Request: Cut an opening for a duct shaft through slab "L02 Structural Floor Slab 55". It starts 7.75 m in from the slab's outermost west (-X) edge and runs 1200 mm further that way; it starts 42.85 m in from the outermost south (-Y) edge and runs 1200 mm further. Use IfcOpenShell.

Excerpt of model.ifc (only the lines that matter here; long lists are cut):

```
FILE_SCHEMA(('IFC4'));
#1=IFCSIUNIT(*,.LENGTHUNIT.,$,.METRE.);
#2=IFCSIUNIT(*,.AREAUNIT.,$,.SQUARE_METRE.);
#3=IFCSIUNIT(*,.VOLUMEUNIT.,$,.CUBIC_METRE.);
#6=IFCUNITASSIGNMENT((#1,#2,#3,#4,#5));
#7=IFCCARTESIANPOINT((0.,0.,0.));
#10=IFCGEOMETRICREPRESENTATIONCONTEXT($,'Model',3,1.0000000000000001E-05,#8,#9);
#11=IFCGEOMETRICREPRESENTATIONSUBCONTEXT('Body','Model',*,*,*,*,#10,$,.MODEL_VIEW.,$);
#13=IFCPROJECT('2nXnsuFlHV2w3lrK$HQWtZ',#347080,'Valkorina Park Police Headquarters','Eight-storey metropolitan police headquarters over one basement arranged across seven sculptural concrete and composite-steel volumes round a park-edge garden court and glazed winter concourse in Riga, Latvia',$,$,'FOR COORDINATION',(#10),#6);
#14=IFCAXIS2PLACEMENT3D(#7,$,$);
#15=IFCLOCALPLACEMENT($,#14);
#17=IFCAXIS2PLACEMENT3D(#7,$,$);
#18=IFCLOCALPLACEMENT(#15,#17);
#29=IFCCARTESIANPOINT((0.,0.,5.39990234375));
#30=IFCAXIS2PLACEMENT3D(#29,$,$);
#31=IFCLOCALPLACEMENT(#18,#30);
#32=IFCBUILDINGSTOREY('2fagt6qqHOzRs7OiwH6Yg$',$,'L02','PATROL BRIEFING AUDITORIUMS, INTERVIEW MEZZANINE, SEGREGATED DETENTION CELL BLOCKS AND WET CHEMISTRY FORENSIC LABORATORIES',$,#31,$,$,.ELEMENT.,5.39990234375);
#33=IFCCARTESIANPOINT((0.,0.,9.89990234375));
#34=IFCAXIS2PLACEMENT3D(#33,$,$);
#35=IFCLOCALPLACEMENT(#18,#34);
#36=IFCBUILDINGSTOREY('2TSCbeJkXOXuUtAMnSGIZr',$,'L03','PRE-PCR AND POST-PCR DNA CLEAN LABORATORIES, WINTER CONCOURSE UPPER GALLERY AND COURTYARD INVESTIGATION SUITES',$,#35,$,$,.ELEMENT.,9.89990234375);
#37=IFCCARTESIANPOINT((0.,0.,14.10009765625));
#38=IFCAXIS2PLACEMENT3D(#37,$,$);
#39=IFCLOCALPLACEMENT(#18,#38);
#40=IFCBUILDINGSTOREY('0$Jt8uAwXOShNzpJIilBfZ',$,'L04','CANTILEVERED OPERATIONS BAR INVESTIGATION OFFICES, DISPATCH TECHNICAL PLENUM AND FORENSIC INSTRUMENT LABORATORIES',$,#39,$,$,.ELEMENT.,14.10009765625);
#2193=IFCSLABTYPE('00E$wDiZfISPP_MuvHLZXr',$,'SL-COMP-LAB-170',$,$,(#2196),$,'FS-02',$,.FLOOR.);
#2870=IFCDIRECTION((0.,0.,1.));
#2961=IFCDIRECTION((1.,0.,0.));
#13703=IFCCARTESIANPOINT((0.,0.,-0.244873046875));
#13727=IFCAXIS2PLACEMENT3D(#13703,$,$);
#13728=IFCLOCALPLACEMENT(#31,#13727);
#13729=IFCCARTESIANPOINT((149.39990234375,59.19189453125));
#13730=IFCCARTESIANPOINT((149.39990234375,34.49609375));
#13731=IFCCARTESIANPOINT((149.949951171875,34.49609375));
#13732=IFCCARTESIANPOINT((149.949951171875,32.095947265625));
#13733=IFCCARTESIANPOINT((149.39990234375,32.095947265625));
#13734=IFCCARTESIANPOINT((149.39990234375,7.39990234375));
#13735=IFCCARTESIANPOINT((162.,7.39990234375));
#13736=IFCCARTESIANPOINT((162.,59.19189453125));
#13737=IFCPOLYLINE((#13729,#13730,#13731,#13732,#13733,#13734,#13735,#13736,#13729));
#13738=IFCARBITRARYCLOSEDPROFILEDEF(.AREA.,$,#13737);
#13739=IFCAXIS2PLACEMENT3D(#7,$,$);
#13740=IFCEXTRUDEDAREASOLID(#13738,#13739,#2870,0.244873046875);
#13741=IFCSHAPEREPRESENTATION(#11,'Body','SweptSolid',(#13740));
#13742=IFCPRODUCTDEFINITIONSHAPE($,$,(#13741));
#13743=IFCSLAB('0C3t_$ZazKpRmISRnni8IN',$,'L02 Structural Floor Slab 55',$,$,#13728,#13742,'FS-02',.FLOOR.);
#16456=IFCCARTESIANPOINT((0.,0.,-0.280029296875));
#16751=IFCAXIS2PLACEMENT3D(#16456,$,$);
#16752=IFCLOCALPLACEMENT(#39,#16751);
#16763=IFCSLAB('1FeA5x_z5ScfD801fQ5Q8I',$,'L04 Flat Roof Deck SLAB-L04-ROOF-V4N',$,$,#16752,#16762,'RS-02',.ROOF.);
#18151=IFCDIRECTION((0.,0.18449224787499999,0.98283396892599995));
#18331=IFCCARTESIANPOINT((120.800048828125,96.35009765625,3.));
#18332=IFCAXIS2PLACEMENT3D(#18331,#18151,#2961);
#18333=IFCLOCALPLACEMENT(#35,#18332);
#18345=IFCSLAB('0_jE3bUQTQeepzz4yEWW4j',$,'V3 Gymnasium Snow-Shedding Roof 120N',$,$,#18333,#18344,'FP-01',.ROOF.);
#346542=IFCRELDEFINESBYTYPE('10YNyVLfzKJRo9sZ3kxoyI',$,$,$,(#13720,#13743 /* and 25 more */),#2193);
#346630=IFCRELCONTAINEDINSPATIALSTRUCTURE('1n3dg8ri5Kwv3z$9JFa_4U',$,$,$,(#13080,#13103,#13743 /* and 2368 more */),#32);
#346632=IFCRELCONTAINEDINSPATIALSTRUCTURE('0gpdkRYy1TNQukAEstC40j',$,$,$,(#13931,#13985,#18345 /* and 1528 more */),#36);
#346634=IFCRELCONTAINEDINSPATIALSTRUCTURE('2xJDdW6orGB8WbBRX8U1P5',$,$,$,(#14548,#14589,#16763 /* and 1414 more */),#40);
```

```python
import numpy as np
import ifcopenshell
import ifcopenshell.api.feature
import ifcopenshell.api.geometry
import ifcopenshell.api.root
import ifcopenshell.geom
import ifcopenshell.util.placement
import ifcopenshell.util.representation
import ifcopenshell.util.shape
import ifcopenshell.util.unit

model = ifcopenshell.open("model.ifc")
unit_scale = ifcopenshell.util.unit.calculate_unit_scale(model)
settings = ifcopenshell.geom.settings()


def volume(element):
    """Net volume in cubic metres, openings subtracted."""
    shape = ifcopenshell.geom.create_shape(settings, element)
    return ifcopenshell.util.shape.get_volume(shape.geometry)


slab = model.by_guid("0C3t_$ZazKpRmISRnni8IN")
before = volume(slab)

# Extent in the slab's own axes, in metres. The edges named are its -X and -Y sides.
slab_shape = ifcopenshell.geom.create_shape(settings, slab)
vertices = ifcopenshell.util.shape.get_vertices(slab_shape.geometry)
x_min, y_min, bottom = vertices.min(axis=0)
top = vertices[:, 2].max()

opening = ifcopenshell.api.root.create_entity(model, ifc_class="IfcOpeningElement", name="Duct shaft opening", predefined_type="OPENING")
context = ifcopenshell.util.representation.get_context(model, "Model", "Body", "MODEL_VIEW")
width, depth = 1.2, 1.2
outline = [(0.0, 0.0), (width, 0.0), (width, depth), (0.0, depth), (0.0, 0.0)]
# Overshoot both faces by 50 mm so the cut is clean.
shape = ifcopenshell.api.geometry.add_slab_representation(
    model, context=context, depth=top - bottom + 0.1, polyline=outline
)
ifcopenshell.api.geometry.assign_representation(model, product=opening, representation=shape)

matrix = ifcopenshell.util.placement.get_local_placement(slab.ObjectPlacement)
matrix[:, 3] = matrix @ np.append(np.array([x_min + 7.75, y_min + 42.85, bottom - 0.05]) / unit_scale, 1.0)
ifcopenshell.api.geometry.edit_object_placement(model, product=opening, matrix=matrix, is_si=False)
ifcopenshell.api.feature.add_feature(model, feature=opening, element=slab)

after = volume(slab)

print(f"slab volume {before:.3f} -> {after:.3f} m3")

model.write("model_v2.ifc")
```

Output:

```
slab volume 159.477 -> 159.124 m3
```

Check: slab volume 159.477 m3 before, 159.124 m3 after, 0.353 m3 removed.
